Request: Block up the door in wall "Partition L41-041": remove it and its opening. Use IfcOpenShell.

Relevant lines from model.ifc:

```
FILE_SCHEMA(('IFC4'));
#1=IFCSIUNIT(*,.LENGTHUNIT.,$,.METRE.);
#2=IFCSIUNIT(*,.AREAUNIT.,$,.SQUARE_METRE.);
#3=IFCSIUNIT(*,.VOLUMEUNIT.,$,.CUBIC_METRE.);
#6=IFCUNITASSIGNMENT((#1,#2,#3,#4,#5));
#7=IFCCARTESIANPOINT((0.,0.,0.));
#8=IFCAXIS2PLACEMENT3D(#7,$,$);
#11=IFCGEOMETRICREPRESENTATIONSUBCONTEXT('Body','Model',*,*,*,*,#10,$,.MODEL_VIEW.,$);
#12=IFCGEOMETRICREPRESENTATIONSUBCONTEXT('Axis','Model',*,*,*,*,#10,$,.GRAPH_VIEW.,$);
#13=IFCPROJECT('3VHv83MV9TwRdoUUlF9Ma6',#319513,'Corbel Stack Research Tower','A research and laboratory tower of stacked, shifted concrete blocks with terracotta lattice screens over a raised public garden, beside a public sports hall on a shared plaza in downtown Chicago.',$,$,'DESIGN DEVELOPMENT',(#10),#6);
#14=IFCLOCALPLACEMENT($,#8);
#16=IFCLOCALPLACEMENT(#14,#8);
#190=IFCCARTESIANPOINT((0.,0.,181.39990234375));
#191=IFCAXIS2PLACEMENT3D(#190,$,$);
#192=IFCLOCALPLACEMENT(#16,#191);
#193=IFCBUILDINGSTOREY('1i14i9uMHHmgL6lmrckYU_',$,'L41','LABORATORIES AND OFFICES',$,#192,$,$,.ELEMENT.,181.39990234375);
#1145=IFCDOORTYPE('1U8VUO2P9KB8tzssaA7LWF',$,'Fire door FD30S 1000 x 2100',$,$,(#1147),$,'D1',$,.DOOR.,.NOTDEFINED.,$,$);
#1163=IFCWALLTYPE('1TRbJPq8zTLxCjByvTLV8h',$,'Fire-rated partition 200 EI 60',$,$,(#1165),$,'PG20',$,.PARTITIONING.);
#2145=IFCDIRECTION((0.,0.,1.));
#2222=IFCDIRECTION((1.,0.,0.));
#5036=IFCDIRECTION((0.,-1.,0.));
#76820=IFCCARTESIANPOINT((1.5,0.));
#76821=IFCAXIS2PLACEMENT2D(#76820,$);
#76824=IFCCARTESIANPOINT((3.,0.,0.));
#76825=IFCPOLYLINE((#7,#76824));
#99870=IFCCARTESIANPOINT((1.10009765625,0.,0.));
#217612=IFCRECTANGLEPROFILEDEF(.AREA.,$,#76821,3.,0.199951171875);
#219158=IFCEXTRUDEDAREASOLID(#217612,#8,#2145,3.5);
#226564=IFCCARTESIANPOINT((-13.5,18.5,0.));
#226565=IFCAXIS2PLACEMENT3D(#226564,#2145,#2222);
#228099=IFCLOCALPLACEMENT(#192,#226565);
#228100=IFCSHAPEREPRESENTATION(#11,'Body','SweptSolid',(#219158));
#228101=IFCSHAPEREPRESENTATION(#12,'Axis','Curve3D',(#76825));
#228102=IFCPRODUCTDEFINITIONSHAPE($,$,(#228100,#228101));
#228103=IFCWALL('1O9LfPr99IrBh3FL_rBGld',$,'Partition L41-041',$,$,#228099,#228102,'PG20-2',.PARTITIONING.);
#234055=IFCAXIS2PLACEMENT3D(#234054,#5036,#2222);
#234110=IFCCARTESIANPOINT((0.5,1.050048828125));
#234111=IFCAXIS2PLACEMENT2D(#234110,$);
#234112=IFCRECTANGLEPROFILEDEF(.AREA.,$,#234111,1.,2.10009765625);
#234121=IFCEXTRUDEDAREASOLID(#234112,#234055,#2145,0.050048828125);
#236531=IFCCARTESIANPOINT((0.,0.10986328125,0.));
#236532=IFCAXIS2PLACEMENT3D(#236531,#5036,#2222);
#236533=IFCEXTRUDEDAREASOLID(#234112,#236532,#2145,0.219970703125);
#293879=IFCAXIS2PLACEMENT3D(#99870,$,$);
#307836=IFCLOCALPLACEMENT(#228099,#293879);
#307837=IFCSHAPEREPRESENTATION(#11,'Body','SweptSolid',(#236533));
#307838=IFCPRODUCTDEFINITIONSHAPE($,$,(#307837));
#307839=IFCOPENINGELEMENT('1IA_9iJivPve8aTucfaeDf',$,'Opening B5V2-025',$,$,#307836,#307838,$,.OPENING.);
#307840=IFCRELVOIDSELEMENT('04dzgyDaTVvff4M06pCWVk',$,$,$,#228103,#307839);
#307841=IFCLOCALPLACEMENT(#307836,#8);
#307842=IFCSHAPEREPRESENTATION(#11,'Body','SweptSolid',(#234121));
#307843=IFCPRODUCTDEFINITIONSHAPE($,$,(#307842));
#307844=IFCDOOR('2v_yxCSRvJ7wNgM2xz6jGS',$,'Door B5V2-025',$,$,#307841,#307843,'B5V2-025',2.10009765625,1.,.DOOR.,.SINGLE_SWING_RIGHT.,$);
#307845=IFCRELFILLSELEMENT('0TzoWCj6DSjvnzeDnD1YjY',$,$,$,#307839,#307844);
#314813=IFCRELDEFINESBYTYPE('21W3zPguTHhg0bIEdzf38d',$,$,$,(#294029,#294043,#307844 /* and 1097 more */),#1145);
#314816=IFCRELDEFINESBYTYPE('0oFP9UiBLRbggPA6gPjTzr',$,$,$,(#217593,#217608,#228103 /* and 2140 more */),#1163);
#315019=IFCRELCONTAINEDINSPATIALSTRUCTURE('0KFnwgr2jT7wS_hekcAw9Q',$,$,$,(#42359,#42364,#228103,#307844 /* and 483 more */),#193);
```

```python
import ifcopenshell
import ifcopenshell.api.feature
import ifcopenshell.api.root
import ifcopenshell.geom
import ifcopenshell.util.shape

model = ifcopenshell.open("model.ifc")
settings = ifcopenshell.geom.settings()


def volume(element):
    """Net volume in cubic metres, openings subtracted."""
    shape = ifcopenshell.geom.create_shape(settings, element)
    return ifcopenshell.util.shape.get_volume(shape.geometry)


door = model.by_id(307844)
opening = door.FillsVoids[0].RelatingOpeningElement
wall = opening.VoidsElements[0].RelatingBuildingElement
before = volume(wall)

ifcopenshell.api.root.remove_product(model, product=door)
ifcopenshell.api.feature.remove_feature(model, feature=opening)

after = volume(wall)

print(f"wall volume {before:.3f} -> {after:.3f} m3")

model.write("model_v2.ifc")
```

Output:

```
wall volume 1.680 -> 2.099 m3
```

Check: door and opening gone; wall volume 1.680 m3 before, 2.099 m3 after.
